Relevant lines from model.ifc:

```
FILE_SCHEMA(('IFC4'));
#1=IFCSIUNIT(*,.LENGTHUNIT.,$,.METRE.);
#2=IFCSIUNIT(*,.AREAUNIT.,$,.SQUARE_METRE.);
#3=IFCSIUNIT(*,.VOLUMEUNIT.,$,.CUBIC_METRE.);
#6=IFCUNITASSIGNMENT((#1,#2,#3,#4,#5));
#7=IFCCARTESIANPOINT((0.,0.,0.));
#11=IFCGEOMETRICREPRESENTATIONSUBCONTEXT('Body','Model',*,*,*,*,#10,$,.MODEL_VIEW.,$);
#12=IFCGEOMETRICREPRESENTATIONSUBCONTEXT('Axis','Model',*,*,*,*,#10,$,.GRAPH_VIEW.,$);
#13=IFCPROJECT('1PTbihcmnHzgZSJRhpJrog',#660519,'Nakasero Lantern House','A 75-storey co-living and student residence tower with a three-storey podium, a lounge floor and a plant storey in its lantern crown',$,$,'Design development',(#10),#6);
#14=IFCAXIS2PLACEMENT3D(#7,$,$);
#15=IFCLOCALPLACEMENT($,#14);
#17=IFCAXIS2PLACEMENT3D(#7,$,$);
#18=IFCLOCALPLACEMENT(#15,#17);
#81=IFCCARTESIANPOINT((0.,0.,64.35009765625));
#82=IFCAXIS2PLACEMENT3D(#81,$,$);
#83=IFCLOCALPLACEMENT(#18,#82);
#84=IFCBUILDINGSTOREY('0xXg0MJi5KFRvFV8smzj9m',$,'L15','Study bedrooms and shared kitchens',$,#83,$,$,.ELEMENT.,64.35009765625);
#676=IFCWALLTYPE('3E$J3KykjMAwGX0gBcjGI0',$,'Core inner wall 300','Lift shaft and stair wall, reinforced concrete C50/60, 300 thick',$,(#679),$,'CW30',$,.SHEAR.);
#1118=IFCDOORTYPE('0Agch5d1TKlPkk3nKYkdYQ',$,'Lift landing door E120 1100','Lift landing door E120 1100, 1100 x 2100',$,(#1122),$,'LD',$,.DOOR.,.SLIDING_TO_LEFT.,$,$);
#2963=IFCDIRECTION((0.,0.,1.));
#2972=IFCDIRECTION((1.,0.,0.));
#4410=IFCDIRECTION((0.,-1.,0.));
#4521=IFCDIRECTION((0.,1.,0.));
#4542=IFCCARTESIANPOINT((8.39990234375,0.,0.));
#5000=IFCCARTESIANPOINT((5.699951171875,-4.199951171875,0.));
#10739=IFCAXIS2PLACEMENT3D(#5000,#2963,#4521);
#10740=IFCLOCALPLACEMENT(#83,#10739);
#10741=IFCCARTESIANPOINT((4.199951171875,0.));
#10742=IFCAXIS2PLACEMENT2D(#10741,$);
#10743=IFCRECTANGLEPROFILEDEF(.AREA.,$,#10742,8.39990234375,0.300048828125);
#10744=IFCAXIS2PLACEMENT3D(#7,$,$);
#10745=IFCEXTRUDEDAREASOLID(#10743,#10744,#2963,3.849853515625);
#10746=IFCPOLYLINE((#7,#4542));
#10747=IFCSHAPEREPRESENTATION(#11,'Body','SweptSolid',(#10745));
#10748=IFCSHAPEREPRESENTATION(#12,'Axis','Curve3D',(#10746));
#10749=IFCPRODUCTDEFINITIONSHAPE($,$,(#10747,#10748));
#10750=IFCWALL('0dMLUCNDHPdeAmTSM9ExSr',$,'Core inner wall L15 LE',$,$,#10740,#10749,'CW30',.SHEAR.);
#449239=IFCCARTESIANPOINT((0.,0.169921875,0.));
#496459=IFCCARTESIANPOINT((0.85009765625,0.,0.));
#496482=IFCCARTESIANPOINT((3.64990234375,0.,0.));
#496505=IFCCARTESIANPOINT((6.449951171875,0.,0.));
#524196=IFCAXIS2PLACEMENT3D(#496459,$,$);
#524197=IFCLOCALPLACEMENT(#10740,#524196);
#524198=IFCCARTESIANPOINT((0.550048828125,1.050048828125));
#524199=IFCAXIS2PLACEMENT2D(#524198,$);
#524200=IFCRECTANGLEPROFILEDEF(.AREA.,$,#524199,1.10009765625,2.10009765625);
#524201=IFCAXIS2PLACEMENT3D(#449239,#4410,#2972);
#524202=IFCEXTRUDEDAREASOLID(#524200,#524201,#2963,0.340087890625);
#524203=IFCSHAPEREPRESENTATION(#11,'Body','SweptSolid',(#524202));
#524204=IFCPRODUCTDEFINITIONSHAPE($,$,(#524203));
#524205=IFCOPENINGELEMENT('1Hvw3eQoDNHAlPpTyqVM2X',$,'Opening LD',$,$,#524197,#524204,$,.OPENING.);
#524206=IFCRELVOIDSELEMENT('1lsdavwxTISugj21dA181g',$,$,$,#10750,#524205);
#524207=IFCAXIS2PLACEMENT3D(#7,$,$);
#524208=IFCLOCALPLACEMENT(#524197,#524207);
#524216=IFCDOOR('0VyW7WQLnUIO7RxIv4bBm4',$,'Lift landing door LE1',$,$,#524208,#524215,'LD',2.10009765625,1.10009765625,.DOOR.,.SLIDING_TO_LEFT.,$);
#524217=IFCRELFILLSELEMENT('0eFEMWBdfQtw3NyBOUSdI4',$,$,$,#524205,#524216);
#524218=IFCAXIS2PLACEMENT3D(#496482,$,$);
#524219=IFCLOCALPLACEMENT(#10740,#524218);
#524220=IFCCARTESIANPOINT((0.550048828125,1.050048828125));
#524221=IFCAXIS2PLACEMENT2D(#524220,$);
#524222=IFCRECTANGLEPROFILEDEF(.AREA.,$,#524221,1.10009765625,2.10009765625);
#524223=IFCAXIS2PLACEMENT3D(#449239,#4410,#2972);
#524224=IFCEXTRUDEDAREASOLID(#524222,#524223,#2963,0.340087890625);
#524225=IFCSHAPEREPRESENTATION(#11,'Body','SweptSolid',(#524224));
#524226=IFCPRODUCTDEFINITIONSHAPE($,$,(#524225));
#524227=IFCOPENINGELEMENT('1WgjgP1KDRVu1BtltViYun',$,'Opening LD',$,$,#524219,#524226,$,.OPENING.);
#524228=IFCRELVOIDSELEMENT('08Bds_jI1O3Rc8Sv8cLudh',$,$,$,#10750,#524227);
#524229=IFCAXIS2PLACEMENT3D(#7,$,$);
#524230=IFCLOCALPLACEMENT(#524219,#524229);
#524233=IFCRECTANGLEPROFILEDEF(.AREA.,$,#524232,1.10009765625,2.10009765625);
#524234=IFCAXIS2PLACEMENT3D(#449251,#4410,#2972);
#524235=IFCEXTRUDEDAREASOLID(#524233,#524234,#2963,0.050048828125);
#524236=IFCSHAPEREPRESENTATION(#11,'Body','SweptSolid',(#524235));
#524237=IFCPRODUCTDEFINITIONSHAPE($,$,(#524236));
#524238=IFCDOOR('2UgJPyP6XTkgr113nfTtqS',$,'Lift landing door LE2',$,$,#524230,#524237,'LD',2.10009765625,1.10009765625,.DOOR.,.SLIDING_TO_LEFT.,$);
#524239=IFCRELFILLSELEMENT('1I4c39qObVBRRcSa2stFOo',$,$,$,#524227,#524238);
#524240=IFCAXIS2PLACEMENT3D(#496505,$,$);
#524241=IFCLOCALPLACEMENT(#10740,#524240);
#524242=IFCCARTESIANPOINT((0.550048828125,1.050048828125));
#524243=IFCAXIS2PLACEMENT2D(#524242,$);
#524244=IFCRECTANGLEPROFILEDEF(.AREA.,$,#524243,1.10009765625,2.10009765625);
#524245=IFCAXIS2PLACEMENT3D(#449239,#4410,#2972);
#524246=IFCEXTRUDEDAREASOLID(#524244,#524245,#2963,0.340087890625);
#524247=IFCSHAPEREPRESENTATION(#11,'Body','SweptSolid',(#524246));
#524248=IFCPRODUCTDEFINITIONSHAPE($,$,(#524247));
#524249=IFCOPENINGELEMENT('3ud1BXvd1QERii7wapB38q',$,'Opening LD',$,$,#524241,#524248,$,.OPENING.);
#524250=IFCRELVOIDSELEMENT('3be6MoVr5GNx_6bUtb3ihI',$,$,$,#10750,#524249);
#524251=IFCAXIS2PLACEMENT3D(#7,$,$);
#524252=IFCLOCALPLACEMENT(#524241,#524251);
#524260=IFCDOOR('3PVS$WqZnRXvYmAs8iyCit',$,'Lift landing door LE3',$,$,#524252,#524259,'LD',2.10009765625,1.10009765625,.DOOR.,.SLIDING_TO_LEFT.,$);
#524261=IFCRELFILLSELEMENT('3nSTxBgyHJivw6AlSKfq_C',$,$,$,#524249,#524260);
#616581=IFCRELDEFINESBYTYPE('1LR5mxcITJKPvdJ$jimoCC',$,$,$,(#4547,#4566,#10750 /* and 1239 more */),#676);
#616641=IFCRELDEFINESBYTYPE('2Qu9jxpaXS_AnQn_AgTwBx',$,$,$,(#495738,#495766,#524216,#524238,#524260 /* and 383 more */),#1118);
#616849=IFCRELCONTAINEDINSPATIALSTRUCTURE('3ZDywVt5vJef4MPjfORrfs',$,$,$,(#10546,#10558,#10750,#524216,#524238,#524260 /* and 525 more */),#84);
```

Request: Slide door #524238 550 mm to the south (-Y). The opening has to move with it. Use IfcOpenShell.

```python
import ifcopenshell
import ifcopenshell.api.geometry
import ifcopenshell.util.placement
import ifcopenshell.util.unit

model = ifcopenshell.open("model.ifc")
unit_scale = ifcopenshell.util.unit.calculate_unit_scale(model)

door = model.by_guid("2UgJPyP6XTkgr113nfTtqS")
opening = door.FillsVoids[0].RelatingOpeningElement
wall = opening.VoidsElements[0].RelatingBuildingElement

wall_matrix = ifcopenshell.util.placement.get_local_placement(wall.ObjectPlacement)
shift = wall_matrix[:3, 0] * -0.55 / unit_scale
before = ifcopenshell.util.placement.get_local_placement(door.ObjectPlacement)[:3, 3].copy()

# The door is placed relative to its opening, so it follows when the opening moves.
matrix = ifcopenshell.util.placement.get_local_placement(opening.ObjectPlacement)
matrix[:3, 3] += shift
ifcopenshell.api.geometry.edit_object_placement(
    model, product=opening, matrix=matrix, is_si=False, should_transform_children=True
)

after = ifcopenshell.util.placement.get_local_placement(door.ObjectPlacement)[:3, 3]
print("door moved by", (after - before).round(3) + 0.0)

model.write("model_updated.ifc")
```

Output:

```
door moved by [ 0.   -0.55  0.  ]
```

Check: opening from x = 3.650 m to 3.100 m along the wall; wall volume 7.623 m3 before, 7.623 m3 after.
